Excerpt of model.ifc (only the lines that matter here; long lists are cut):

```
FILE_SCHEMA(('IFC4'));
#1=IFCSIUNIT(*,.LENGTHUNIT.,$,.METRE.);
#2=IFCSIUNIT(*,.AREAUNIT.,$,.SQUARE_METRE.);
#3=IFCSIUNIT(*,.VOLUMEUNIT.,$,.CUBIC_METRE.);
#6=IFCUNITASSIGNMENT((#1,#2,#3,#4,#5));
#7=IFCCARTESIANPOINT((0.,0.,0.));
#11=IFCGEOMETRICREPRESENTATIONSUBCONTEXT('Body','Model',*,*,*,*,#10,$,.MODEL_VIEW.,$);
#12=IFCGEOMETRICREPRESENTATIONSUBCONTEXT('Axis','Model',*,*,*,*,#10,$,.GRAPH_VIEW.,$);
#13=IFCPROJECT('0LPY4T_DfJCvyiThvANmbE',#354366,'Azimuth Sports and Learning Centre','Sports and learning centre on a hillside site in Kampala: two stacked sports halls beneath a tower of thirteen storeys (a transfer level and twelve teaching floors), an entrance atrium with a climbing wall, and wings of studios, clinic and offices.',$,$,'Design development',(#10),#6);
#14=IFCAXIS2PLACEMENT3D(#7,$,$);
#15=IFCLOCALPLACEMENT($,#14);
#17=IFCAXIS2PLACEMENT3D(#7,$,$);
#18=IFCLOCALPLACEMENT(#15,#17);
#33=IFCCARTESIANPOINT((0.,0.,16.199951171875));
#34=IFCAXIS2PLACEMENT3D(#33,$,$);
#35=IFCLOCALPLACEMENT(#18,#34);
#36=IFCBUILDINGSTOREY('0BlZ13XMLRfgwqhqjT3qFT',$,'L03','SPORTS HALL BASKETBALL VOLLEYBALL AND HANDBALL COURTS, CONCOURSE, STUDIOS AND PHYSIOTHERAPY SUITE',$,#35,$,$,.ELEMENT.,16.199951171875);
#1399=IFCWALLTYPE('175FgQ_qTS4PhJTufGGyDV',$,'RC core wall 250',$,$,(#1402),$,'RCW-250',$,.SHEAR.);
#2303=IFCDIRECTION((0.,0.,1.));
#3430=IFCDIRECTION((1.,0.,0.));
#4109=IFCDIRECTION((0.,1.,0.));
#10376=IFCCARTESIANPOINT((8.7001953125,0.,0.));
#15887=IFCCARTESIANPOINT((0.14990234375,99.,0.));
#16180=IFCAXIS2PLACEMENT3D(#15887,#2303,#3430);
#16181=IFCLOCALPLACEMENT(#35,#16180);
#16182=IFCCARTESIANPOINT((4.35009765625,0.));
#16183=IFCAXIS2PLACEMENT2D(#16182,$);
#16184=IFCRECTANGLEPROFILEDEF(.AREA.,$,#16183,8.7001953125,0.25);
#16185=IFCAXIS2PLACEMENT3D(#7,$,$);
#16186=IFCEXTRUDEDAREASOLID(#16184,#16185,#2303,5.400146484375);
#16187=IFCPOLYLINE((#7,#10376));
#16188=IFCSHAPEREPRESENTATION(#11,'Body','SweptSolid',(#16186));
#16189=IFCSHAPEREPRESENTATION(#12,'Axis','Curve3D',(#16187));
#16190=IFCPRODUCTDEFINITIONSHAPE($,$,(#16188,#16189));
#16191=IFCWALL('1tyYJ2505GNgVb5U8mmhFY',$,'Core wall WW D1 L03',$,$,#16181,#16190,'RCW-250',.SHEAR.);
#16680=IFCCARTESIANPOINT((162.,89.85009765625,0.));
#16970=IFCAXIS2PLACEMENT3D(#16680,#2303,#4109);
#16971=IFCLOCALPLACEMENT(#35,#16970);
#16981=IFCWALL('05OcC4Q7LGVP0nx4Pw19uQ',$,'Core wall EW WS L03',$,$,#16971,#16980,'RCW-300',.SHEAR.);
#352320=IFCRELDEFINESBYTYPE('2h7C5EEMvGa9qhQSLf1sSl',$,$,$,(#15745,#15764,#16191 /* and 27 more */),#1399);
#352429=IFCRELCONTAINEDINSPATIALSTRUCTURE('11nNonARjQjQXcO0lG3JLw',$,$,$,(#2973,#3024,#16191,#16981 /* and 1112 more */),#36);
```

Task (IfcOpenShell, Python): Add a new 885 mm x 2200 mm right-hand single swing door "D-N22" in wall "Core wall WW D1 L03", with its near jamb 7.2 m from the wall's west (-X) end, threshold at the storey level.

```python
import numpy as np
import ifcopenshell
import ifcopenshell.api.feature
import ifcopenshell.api.geometry
import ifcopenshell.api.root
import ifcopenshell.api.spatial
import ifcopenshell.geom
import ifcopenshell.util.element
import ifcopenshell.util.placement
import ifcopenshell.util.representation
import ifcopenshell.util.shape
import ifcopenshell.util.unit

model = ifcopenshell.open("model.ifc")
unit_scale = ifcopenshell.util.unit.calculate_unit_scale(model)
settings = ifcopenshell.geom.settings()


def volume(element):
    """Net volume in cubic metres, openings subtracted."""
    shape = ifcopenshell.geom.create_shape(settings, element)
    return ifcopenshell.util.shape.get_volume(shape.geometry)


wall = model.by_id(16191)
storey = ifcopenshell.util.element.get_container(wall, ifc_class="IfcBuildingStorey")
context = ifcopenshell.util.representation.get_context(model, "Model", "Body", "MODEL_VIEW")
before = volume(wall)

width, height, from_end, sill = 0.885, 2.2, 7.2, 0.0  # metres

# The wall runs along its own X axis, and the end named is its -X end.
wall_shape = ifcopenshell.geom.create_shape(settings, wall)
x, y, z = ifcopenshell.util.shape.get_vertices(wall_shape.geometry).T
start = x.min() + from_end
face, thickness = float(y.min()), float(y.max() - y.min())
wall_matrix = ifcopenshell.util.placement.get_local_placement(wall.ObjectPlacement)
level = ifcopenshell.util.placement.get_local_placement(storey.ObjectPlacement)[2, 3]


def in_wall(x, y):
    """Placement at x, y metres in the wall's axes, at sill height."""
    matrix = wall_matrix.copy()
    matrix[:, 3] = wall_matrix @ np.array([x / unit_scale, y / unit_scale, 0.0, 1.0])
    matrix[2, 3] = level + sill / unit_scale
    return matrix


# Opening: a box that overshoots both wall faces by 50 mm.
opening = ifcopenshell.api.root.create_entity(model, ifc_class="IfcOpeningElement", predefined_type="OPENING")
box = ifcopenshell.api.geometry.add_wall_representation(
    model, context=context, length=width, height=height, thickness=thickness + 0.1
)
ifcopenshell.api.geometry.assign_representation(model, product=opening, representation=box)
ifcopenshell.api.geometry.edit_object_placement(model, product=opening, matrix=in_wall(start, face - 0.05), is_si=False)
ifcopenshell.api.feature.add_feature(model, feature=opening, element=wall)

door = ifcopenshell.api.root.create_entity(model, ifc_class="IfcDoor", name="D-N22", predefined_type="DOOR")
door.OverallWidth, door.OverallHeight = width / unit_scale, height / unit_scale
door.OperationType = "SINGLE_SWING_RIGHT"
body = ifcopenshell.api.geometry.add_door_representation(
    model,
    context=context,
    overall_width=door.OverallWidth,
    overall_height=door.OverallHeight,
    operation_type="SINGLE_SWING_RIGHT",
    lining_properties={"LiningDepth": thickness / unit_scale, "ThresholdDepth": thickness / unit_scale},
)
ifcopenshell.api.geometry.assign_representation(model, product=door, representation=body)
ifcopenshell.api.spatial.assign_container(model, products=[door], relating_structure=storey)
ifcopenshell.api.feature.add_filling(model, opening=opening, element=door)

# The lining spans the wall, so the door starts at the wall face.
ifcopenshell.api.geometry.edit_object_placement(model, product=door, matrix=in_wall(start, face), is_si=False)

after = volume(wall)

print(f"wall volume {before:.3f} -> {after:.3f} m3")

model.write("model_v2.ifc")
```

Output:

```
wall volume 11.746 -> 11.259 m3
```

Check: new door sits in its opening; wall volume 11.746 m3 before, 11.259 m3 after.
